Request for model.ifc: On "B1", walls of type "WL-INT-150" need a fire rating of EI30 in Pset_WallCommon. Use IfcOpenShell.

First a look at what the model holds.

```python
import ifcopenshell
import ifcopenshell.util.element

model = ifcopenshell.open("model.ifc")
print(model.schema)
storey = next(s for s in model.by_type("IfcBuildingStorey") if s.Name == "B1")
walls = [e for e in ifcopenshell.util.element.get_decomposition(storey) if e.is_a("IfcWall")]
seen = {}
for e in walls:
    element_type = ifcopenshell.util.element.get_type(e)
    key = (element_type.Name if element_type != e and element_type else None, ifcopenshell.util.element.get_pset(e, "Pset_WallCommon", "FireRating"))
    seen[key] = seen.get(key, 0) + 1
for (name, value), count in sorted(seen.items(), key=str):
    print(count, "x", name, "|", value)
```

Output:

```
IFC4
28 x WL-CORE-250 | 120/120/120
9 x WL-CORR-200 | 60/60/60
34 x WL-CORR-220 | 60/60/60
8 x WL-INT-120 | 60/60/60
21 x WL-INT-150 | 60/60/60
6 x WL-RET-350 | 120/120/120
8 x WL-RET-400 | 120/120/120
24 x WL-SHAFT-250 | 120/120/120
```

```python
import ifcopenshell
import ifcopenshell.api.pset
import ifcopenshell.util.element

model = ifcopenshell.open("model.ifc")

storey = next(s for s in model.by_type("IfcBuildingStorey") if s.Name == "B1")
walls = [e for e in ifcopenshell.util.element.get_decomposition(storey) if e.is_a("IfcWall")]

count = 0
for e in walls:
    element_type = ifcopenshell.util.element.get_type(e)
    if element_type in (None, e) or element_type.Name != "WL-INT-150":
        continue
    # add_pset returns the element's existing set when there is one.
    pset = ifcopenshell.api.pset.add_pset(model, product=e, name="Pset_WallCommon")
    ifcopenshell.api.pset.edit_pset(model, pset=pset, properties={"FireRating": "EI30"})
    count += 1

print(count, "walls updated")

model.write("model_v2.ifc")
```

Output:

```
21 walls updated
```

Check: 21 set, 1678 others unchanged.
